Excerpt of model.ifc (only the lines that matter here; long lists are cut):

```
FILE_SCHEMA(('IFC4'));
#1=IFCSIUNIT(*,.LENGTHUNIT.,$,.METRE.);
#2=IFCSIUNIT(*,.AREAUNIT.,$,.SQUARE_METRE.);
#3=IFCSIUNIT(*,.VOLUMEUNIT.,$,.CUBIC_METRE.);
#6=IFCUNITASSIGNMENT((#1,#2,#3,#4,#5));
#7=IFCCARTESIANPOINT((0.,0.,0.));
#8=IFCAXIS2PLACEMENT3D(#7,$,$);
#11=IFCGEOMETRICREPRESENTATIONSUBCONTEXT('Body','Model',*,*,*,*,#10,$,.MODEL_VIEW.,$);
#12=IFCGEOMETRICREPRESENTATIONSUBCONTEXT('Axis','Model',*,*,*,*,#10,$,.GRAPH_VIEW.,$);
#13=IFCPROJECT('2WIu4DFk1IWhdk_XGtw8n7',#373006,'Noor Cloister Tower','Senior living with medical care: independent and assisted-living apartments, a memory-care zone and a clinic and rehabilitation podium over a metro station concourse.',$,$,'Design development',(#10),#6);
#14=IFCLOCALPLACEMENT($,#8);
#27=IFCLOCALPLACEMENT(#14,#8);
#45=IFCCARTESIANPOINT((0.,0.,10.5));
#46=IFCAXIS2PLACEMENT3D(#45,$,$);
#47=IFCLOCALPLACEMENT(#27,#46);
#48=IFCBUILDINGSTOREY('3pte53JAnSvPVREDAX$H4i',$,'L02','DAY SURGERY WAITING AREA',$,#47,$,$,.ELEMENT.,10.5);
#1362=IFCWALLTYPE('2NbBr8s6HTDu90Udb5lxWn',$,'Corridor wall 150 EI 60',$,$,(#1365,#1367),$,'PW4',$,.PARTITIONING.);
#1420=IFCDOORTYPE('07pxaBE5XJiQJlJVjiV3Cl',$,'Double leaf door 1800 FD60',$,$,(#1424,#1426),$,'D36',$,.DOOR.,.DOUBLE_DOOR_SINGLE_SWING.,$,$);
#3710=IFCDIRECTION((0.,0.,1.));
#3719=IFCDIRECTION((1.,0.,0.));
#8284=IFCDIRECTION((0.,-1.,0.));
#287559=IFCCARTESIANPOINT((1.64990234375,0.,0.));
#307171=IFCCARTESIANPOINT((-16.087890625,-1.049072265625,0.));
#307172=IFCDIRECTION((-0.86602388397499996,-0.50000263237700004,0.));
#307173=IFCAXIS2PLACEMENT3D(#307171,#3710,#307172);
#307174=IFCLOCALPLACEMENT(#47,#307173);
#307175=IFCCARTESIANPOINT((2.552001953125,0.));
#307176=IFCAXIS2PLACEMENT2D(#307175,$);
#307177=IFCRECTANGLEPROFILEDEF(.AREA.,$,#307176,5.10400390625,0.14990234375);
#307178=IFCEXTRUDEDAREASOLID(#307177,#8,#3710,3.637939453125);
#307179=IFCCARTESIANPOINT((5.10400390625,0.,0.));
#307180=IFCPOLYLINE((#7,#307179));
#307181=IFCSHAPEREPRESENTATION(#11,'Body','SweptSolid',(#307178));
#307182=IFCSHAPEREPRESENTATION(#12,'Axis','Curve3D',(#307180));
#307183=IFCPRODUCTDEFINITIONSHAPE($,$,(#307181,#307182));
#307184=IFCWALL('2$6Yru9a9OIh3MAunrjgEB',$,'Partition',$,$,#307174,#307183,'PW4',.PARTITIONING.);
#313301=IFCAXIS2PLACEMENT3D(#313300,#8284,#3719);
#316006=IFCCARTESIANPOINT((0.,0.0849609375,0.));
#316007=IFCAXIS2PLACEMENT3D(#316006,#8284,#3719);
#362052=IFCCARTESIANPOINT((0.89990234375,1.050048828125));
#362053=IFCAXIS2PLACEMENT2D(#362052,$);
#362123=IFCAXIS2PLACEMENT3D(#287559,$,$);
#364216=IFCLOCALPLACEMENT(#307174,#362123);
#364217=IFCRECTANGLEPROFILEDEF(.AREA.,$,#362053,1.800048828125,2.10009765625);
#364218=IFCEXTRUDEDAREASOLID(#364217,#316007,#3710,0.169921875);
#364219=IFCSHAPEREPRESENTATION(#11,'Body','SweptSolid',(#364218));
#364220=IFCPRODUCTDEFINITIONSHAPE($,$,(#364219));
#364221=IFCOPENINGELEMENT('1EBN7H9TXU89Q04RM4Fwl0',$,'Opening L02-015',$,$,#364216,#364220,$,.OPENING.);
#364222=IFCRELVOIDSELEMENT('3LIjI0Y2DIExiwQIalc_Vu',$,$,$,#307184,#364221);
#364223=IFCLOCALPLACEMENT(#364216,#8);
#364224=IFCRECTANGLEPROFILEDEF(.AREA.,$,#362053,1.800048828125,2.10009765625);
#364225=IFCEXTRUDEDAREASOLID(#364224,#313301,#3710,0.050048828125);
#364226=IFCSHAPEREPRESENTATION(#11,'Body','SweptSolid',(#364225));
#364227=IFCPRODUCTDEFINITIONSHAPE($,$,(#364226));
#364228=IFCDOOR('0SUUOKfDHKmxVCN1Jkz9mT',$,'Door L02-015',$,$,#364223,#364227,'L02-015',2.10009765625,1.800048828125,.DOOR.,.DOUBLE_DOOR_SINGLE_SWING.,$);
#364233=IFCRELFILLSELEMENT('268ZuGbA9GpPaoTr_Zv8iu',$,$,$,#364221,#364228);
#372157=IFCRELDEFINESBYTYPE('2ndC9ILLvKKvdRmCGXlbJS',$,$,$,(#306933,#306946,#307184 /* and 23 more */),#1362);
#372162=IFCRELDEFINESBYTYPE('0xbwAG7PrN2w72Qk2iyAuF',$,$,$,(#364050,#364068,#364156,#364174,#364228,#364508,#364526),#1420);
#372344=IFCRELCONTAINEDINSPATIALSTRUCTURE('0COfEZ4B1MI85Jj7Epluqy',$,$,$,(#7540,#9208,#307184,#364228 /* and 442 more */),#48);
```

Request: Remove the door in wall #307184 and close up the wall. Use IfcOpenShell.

```python
import ifcopenshell
import ifcopenshell.api.feature
import ifcopenshell.api.root
import ifcopenshell.geom
import ifcopenshell.util.shape

model = ifcopenshell.open("model.ifc")
settings = ifcopenshell.geom.settings()


def volume(element):
    """Net volume in cubic metres, openings subtracted."""
    shape = ifcopenshell.geom.create_shape(settings, element)
    return ifcopenshell.util.shape.get_volume(shape.geometry)


door = model.by_guid("0SUUOKfDHKmxVCN1Jkz9mT")
opening = door.FillsVoids[0].RelatingOpeningElement
wall = opening.VoidsElements[0].RelatingBuildingElement
before = volume(wall)

ifcopenshell.api.root.remove_product(model, product=door)
ifcopenshell.api.feature.remove_feature(model, feature=opening)

after = volume(wall)

print(f"wall volume {before:.3f} -> {after:.3f} m3")

model.write("model_v2.ifc")
```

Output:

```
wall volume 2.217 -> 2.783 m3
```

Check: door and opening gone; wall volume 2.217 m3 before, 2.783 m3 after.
